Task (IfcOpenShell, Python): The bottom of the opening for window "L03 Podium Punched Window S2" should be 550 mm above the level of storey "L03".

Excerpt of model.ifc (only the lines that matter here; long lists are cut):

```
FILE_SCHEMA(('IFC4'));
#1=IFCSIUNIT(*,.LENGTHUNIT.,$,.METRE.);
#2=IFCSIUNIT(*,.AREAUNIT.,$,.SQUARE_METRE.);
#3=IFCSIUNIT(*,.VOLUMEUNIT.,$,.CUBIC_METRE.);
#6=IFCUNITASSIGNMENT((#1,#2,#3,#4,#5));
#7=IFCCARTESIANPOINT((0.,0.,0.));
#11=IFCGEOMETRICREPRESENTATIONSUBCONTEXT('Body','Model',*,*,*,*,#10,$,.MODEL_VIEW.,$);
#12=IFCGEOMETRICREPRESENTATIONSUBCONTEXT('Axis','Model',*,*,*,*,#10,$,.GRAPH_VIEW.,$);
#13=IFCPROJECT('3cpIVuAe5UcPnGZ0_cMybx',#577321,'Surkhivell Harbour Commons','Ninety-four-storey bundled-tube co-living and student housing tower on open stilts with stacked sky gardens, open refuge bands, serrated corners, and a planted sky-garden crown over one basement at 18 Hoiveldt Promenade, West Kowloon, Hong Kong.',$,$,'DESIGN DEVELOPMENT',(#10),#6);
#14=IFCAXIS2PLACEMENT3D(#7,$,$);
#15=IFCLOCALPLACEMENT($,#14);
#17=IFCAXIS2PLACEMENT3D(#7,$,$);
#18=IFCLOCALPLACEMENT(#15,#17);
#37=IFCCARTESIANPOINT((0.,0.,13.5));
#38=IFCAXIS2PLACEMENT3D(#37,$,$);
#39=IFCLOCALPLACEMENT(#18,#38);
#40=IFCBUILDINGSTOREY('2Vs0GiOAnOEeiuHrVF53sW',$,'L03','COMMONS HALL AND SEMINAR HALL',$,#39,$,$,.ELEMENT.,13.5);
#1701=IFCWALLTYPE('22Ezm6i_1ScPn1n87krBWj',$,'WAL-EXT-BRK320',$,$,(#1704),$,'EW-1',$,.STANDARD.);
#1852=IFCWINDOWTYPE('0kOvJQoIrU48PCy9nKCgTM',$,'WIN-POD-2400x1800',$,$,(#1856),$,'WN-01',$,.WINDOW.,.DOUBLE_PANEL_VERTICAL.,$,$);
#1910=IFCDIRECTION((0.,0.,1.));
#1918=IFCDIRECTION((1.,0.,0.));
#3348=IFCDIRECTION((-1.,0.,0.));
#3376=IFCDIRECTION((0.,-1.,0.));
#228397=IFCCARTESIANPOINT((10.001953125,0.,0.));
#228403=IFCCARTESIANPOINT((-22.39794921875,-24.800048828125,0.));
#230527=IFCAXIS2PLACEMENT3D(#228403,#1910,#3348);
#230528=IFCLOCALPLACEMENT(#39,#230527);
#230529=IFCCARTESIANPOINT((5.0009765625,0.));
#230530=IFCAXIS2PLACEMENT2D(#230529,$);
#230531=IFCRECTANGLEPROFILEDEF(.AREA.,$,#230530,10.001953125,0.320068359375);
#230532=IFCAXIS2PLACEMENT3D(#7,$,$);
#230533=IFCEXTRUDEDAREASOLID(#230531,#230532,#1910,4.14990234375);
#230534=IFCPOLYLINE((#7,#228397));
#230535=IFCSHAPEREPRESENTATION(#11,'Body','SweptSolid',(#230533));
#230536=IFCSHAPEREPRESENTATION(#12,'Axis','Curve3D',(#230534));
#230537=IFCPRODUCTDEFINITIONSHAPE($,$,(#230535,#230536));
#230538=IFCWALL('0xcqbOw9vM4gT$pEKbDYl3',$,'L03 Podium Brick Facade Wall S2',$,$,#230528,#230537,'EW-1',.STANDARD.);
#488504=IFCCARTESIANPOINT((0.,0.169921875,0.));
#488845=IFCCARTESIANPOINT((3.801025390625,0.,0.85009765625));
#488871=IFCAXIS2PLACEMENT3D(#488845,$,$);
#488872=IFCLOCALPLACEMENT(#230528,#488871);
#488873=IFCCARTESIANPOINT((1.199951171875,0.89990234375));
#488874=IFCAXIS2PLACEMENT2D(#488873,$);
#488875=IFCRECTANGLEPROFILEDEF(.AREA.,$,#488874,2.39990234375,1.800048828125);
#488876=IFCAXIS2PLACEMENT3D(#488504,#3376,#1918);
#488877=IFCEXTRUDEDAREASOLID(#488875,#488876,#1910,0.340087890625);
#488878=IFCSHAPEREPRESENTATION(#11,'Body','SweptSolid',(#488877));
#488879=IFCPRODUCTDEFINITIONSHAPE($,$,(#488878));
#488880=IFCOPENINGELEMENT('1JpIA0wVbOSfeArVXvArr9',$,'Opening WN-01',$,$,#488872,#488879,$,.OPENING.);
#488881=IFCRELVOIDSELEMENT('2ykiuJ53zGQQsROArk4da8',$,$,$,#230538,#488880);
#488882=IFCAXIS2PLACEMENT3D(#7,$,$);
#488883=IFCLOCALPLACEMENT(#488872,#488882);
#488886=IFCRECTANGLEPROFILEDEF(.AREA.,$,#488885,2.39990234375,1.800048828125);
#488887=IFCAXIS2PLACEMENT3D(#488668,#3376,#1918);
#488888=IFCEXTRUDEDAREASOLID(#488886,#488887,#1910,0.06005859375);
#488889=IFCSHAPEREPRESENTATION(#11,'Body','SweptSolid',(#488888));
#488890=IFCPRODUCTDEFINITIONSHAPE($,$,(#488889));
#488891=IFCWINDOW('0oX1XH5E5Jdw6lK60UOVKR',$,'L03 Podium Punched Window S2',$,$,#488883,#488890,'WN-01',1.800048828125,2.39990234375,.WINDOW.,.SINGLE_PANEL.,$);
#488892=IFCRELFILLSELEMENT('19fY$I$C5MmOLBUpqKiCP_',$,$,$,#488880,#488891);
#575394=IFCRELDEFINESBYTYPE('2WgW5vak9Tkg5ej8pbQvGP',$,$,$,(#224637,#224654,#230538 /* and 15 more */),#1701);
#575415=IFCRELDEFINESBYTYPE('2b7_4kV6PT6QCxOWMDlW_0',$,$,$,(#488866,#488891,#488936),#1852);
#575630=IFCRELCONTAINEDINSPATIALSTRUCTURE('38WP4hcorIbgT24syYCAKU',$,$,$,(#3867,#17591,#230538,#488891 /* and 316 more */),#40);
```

```python
import numpy as np
import ifcopenshell
import ifcopenshell.api.geometry
import ifcopenshell.geom
import ifcopenshell.util.element
import ifcopenshell.util.placement
import ifcopenshell.util.shape
import ifcopenshell.util.unit

model = ifcopenshell.open("model.ifc")
unit_scale = ifcopenshell.util.unit.calculate_unit_scale(model)

window = model.by_guid("0oX1XH5E5Jdw6lK60UOVKR")
opening = window.FillsVoids[0].RelatingOpeningElement
storey = ifcopenshell.util.element.get_container(window, ifc_class="IfcBuildingStorey")
level = ifcopenshell.util.placement.get_local_placement(storey.ObjectPlacement)[2, 3]

# The opening's origin need not be at the sill, so measure its lowest point.
shape = ifcopenshell.geom.create_shape(ifcopenshell.geom.settings(), opening)
bottom = ifcopenshell.util.shape.get_shape_bottom_elevation(shape, shape.geometry) / unit_scale
dz = level + 0.55 / unit_scale - bottom

shift = np.array([0.0, 0.0, dz])
# The window is placed relative to its opening, so it follows when the opening moves.
matrix = ifcopenshell.util.placement.get_local_placement(opening.ObjectPlacement)
matrix[:3, 3] += shift
ifcopenshell.api.geometry.edit_object_placement(
    model, product=opening, matrix=matrix, is_si=False, should_transform_children=True
)

print(f"moved by {dz * unit_scale:+.3f} m")

model.write("model-out.ifc")
```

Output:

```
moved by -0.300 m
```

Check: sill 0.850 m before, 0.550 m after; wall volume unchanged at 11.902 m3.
